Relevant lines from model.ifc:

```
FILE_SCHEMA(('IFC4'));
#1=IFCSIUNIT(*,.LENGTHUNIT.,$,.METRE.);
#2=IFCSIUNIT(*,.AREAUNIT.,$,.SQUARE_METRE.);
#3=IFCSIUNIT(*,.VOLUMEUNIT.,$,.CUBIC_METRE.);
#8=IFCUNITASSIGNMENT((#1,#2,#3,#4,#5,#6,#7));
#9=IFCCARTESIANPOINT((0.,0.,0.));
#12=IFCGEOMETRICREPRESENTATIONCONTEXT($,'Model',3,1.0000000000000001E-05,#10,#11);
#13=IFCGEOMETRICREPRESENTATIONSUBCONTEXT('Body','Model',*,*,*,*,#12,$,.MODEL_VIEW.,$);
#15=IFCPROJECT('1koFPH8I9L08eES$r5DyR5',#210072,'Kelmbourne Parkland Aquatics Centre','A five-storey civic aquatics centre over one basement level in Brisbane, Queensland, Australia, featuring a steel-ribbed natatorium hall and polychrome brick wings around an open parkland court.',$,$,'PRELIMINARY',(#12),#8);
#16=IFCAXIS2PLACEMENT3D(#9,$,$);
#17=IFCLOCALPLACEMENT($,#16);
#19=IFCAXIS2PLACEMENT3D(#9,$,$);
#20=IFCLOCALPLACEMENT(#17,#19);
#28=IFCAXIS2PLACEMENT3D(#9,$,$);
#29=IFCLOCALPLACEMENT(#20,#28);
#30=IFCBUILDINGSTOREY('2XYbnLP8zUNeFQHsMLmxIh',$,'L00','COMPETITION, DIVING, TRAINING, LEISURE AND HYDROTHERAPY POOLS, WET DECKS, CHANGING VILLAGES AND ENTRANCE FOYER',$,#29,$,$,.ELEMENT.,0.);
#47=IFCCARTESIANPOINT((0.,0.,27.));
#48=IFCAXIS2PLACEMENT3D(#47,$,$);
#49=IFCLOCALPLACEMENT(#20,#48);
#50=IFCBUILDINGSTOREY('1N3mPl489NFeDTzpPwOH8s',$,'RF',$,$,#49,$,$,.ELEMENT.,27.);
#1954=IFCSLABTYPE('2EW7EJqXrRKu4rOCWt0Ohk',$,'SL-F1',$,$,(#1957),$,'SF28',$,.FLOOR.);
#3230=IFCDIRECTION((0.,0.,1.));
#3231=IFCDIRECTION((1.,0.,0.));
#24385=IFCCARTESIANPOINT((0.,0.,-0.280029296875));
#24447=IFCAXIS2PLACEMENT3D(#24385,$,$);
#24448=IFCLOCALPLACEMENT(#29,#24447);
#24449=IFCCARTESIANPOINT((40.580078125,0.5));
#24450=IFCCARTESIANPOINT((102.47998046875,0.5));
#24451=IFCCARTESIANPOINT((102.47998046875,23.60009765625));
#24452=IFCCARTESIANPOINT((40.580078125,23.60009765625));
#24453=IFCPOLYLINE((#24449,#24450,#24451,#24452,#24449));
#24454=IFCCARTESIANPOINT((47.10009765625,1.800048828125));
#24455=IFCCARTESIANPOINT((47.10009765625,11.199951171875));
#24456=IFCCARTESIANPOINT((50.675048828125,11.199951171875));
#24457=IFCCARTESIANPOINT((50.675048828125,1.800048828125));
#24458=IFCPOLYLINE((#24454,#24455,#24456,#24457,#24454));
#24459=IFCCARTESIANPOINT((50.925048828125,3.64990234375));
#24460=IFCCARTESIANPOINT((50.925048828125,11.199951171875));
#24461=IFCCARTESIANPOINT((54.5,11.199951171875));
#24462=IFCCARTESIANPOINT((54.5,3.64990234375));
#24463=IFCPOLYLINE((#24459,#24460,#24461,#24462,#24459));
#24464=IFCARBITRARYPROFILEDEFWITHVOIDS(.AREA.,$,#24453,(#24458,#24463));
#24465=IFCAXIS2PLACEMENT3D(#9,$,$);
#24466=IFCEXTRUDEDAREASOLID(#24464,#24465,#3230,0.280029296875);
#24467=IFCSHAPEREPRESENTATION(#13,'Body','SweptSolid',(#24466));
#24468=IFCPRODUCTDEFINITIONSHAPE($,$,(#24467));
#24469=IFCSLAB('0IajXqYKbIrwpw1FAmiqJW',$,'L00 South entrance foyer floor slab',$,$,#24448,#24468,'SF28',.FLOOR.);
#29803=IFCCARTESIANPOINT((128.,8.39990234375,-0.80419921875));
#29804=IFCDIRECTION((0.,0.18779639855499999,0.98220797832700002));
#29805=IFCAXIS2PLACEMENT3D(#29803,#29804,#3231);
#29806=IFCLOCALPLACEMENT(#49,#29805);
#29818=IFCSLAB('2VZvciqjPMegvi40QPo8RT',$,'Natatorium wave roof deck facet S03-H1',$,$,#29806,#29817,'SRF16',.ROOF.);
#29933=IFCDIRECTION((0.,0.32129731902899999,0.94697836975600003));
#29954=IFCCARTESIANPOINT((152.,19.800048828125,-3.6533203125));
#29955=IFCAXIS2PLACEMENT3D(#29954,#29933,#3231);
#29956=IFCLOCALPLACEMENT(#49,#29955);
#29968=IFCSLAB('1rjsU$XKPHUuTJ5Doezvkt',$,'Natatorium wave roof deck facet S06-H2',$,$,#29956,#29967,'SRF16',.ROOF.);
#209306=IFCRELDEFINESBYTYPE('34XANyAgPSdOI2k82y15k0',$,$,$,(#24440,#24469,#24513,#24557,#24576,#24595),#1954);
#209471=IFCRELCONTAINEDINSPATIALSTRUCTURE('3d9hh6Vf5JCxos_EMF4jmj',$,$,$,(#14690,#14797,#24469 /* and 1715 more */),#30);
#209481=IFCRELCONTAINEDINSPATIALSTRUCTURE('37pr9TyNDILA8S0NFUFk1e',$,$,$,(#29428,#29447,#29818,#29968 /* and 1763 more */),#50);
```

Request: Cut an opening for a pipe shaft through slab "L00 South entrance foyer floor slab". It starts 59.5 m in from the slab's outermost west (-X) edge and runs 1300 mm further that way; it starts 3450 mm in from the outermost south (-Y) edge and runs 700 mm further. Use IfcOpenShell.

```python
import numpy as np
import ifcopenshell
import ifcopenshell.api.feature
import ifcopenshell.api.geometry
import ifcopenshell.api.root
import ifcopenshell.geom
import ifcopenshell.util.placement
import ifcopenshell.util.representation
import ifcopenshell.util.shape
import ifcopenshell.util.unit

model = ifcopenshell.open("model.ifc")
unit_scale = ifcopenshell.util.unit.calculate_unit_scale(model)
settings = ifcopenshell.geom.settings()


def volume(element):
    """Net volume in cubic metres, openings subtracted."""
    shape = ifcopenshell.geom.create_shape(settings, element)
    return ifcopenshell.util.shape.get_volume(shape.geometry)


slab = model.by_guid("0IajXqYKbIrwpw1FAmiqJW")
before = volume(slab)

# Extent in the slab's own axes, in metres. The edges named are its -X and -Y sides.
slab_shape = ifcopenshell.geom.create_shape(settings, slab)
vertices = ifcopenshell.util.shape.get_vertices(slab_shape.geometry)
x_min, y_min, bottom = vertices.min(axis=0)
top = vertices[:, 2].max()

opening = ifcopenshell.api.root.create_entity(model, ifc_class="IfcOpeningElement", name="Pipe shaft opening", predefined_type="OPENING")
context = ifcopenshell.util.representation.get_context(model, "Model", "Body", "MODEL_VIEW")
width, depth = 1.3, 0.7
outline = [(0.0, 0.0), (width, 0.0), (width, depth), (0.0, depth), (0.0, 0.0)]
# Overshoot both faces by 50 mm so the cut is clean.
shape = ifcopenshell.api.geometry.add_slab_representation(
    model, context=context, depth=top - bottom + 0.1, polyline=outline
)
ifcopenshell.api.geometry.assign_representation(model, product=opening, representation=shape)

matrix = ifcopenshell.util.placement.get_local_placement(slab.ObjectPlacement)
matrix[:, 3] = matrix @ np.append(np.array([x_min + 59.5, y_min + 3.45, bottom - 0.05]) / unit_scale, 1.0)
ifcopenshell.api.geometry.edit_object_placement(model, product=opening, matrix=matrix, is_si=False)
ifcopenshell.api.feature.add_feature(model, feature=opening, element=slab)

after = volume(slab)

print(f"slab volume {before:.3f} -> {after:.3f} m3")

model.write("model_edited.ifc")
```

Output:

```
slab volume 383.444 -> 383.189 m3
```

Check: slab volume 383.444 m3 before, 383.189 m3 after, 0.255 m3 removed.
